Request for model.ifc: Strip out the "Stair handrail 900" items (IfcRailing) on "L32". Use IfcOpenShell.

First a look at what the model holds.

```python
import ifcopenshell
import ifcopenshell.util.element

model = ifcopenshell.open("model.ifc")
print(model.schema)
storey = next(s for s in model.by_type("IfcBuildingStorey") if s.Name == "L32")
railings = [e for e in ifcopenshell.util.element.get_decomposition(storey) if e.is_a("IfcRailing")]
seen = {}
for e in railings:
    element_type = ifcopenshell.util.element.get_type(e)
    name = element_type.Name if element_type not in (None, e) else None
    seen[name] = seen.get(name, 0) + 1
for name, count in sorted(seen.items(), key=str):
    print(count, "x", name)
```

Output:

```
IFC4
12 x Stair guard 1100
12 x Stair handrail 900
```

```python
import ifcopenshell
import ifcopenshell.api.root
import ifcopenshell.util.element

model = ifcopenshell.open("model.ifc")

storey = next(s for s in model.by_type("IfcBuildingStorey") if s.Name == "L32")
railings = [e for e in ifcopenshell.util.element.get_decomposition(storey) if e.is_a("IfcRailing")]
targets = [e for e in railings if (t := ifcopenshell.util.element.get_type(e)) not in (None, e) and t.Name == "Stair handrail 900"]

for e in targets:
    ifcopenshell.api.root.remove_product(model, product=e)
print(len(targets), "removed")

model.write("model_edited.ifc")
```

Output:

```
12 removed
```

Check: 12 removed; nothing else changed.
